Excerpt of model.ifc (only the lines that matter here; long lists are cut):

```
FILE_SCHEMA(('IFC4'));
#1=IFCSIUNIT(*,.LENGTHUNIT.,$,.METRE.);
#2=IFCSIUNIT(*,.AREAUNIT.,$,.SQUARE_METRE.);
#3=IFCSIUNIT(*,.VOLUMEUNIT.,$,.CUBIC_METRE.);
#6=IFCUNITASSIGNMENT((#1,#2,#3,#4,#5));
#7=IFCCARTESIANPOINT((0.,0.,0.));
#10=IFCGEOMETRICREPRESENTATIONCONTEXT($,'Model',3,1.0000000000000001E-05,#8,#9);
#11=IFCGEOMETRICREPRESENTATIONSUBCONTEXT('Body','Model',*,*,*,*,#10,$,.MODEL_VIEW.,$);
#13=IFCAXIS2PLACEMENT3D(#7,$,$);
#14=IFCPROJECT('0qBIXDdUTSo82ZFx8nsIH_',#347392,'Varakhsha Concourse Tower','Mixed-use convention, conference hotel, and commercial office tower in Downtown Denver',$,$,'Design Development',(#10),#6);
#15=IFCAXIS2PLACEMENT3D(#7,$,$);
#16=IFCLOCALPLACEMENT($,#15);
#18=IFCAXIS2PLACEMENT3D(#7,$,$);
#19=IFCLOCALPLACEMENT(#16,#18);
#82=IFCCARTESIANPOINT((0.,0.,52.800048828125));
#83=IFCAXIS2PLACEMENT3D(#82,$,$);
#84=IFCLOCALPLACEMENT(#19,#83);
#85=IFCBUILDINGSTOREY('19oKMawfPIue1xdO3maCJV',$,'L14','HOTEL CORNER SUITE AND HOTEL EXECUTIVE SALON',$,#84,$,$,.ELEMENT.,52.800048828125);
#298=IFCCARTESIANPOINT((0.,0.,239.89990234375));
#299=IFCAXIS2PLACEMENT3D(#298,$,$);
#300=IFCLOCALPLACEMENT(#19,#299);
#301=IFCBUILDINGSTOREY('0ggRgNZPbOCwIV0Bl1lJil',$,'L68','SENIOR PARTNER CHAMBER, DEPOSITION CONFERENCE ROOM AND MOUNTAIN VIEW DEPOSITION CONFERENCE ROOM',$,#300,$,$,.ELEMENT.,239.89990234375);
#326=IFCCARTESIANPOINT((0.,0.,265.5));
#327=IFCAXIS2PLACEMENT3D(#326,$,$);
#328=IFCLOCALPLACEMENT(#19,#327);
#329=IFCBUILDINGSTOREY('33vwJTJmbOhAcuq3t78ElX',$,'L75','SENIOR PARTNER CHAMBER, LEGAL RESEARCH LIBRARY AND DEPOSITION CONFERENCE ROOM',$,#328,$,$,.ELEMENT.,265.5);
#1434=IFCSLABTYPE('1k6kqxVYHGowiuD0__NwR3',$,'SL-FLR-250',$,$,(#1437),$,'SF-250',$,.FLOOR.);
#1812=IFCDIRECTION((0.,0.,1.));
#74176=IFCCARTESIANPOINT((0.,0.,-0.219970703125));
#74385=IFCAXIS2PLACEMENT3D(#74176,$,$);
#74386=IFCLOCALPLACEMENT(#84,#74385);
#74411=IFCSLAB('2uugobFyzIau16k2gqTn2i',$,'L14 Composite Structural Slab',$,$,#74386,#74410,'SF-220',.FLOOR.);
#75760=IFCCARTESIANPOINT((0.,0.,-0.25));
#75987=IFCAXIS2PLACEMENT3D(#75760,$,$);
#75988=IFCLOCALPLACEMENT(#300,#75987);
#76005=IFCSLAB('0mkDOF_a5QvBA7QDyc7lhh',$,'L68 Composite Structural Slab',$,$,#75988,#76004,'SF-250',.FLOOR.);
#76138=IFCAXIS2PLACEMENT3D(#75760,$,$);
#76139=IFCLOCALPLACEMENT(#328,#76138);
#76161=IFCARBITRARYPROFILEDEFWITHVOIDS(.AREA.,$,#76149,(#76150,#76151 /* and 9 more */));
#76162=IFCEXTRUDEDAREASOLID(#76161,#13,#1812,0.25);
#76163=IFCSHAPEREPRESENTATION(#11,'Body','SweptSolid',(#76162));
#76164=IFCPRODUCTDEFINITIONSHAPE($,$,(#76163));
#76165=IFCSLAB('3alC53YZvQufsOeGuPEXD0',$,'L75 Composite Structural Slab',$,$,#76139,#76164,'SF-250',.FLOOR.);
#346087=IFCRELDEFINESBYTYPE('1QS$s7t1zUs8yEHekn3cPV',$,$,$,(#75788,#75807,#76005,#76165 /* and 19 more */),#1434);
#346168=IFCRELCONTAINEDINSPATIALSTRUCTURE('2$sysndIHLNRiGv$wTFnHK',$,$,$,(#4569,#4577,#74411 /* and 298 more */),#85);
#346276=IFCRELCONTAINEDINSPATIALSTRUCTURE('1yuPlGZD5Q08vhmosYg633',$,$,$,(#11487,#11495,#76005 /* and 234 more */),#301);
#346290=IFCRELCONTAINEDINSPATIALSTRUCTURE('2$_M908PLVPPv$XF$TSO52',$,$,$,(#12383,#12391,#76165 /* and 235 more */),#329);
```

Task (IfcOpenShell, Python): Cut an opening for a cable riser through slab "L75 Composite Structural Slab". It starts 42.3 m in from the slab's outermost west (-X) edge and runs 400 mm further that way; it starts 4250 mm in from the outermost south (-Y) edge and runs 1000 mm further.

```python
import numpy as np
import ifcopenshell
import ifcopenshell.api.feature
import ifcopenshell.api.geometry
import ifcopenshell.api.root
import ifcopenshell.geom
import ifcopenshell.util.placement
import ifcopenshell.util.representation
import ifcopenshell.util.shape
import ifcopenshell.util.unit

model = ifcopenshell.open("model.ifc")
unit_scale = ifcopenshell.util.unit.calculate_unit_scale(model)
settings = ifcopenshell.geom.settings()


def volume(element):
    """Net volume in cubic metres, openings subtracted."""
    shape = ifcopenshell.geom.create_shape(settings, element)
    return ifcopenshell.util.shape.get_volume(shape.geometry)


slab = model.by_guid("3alC53YZvQufsOeGuPEXD0")
before = volume(slab)

# Extent in the slab's own axes, in metres. The edges named are its -X and -Y sides.
slab_shape = ifcopenshell.geom.create_shape(settings, slab)
vertices = ifcopenshell.util.shape.get_vertices(slab_shape.geometry)
x_min, y_min, bottom = vertices.min(axis=0)
top = vertices[:, 2].max()

opening = ifcopenshell.api.root.create_entity(model, ifc_class="IfcOpeningElement", name="Cable riser opening", predefined_type="OPENING")
context = ifcopenshell.util.representation.get_context(model, "Model", "Body", "MODEL_VIEW")
width, depth = 0.4, 1
outline = [(0.0, 0.0), (width, 0.0), (width, depth), (0.0, depth), (0.0, 0.0)]
# Overshoot both faces by 50 mm so the cut is clean.
shape = ifcopenshell.api.geometry.add_slab_representation(
    model, context=context, depth=top - bottom + 0.1, polyline=outline
)
ifcopenshell.api.geometry.assign_representation(model, product=opening, representation=shape)

matrix = ifcopenshell.util.placement.get_local_placement(slab.ObjectPlacement)
matrix[:, 3] = matrix @ np.append(np.array([x_min + 42.3, y_min + 4.25, bottom - 0.05]) / unit_scale, 1.0)
ifcopenshell.api.geometry.edit_object_placement(model, product=opening, matrix=matrix, is_si=False)
ifcopenshell.api.feature.add_feature(model, feature=opening, element=slab)

after = volume(slab)

print(f"slab volume {before:.3f} -> {after:.3f} m3")

model.write("model-out.ifc")
```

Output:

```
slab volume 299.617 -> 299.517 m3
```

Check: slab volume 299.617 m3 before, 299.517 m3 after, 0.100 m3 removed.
